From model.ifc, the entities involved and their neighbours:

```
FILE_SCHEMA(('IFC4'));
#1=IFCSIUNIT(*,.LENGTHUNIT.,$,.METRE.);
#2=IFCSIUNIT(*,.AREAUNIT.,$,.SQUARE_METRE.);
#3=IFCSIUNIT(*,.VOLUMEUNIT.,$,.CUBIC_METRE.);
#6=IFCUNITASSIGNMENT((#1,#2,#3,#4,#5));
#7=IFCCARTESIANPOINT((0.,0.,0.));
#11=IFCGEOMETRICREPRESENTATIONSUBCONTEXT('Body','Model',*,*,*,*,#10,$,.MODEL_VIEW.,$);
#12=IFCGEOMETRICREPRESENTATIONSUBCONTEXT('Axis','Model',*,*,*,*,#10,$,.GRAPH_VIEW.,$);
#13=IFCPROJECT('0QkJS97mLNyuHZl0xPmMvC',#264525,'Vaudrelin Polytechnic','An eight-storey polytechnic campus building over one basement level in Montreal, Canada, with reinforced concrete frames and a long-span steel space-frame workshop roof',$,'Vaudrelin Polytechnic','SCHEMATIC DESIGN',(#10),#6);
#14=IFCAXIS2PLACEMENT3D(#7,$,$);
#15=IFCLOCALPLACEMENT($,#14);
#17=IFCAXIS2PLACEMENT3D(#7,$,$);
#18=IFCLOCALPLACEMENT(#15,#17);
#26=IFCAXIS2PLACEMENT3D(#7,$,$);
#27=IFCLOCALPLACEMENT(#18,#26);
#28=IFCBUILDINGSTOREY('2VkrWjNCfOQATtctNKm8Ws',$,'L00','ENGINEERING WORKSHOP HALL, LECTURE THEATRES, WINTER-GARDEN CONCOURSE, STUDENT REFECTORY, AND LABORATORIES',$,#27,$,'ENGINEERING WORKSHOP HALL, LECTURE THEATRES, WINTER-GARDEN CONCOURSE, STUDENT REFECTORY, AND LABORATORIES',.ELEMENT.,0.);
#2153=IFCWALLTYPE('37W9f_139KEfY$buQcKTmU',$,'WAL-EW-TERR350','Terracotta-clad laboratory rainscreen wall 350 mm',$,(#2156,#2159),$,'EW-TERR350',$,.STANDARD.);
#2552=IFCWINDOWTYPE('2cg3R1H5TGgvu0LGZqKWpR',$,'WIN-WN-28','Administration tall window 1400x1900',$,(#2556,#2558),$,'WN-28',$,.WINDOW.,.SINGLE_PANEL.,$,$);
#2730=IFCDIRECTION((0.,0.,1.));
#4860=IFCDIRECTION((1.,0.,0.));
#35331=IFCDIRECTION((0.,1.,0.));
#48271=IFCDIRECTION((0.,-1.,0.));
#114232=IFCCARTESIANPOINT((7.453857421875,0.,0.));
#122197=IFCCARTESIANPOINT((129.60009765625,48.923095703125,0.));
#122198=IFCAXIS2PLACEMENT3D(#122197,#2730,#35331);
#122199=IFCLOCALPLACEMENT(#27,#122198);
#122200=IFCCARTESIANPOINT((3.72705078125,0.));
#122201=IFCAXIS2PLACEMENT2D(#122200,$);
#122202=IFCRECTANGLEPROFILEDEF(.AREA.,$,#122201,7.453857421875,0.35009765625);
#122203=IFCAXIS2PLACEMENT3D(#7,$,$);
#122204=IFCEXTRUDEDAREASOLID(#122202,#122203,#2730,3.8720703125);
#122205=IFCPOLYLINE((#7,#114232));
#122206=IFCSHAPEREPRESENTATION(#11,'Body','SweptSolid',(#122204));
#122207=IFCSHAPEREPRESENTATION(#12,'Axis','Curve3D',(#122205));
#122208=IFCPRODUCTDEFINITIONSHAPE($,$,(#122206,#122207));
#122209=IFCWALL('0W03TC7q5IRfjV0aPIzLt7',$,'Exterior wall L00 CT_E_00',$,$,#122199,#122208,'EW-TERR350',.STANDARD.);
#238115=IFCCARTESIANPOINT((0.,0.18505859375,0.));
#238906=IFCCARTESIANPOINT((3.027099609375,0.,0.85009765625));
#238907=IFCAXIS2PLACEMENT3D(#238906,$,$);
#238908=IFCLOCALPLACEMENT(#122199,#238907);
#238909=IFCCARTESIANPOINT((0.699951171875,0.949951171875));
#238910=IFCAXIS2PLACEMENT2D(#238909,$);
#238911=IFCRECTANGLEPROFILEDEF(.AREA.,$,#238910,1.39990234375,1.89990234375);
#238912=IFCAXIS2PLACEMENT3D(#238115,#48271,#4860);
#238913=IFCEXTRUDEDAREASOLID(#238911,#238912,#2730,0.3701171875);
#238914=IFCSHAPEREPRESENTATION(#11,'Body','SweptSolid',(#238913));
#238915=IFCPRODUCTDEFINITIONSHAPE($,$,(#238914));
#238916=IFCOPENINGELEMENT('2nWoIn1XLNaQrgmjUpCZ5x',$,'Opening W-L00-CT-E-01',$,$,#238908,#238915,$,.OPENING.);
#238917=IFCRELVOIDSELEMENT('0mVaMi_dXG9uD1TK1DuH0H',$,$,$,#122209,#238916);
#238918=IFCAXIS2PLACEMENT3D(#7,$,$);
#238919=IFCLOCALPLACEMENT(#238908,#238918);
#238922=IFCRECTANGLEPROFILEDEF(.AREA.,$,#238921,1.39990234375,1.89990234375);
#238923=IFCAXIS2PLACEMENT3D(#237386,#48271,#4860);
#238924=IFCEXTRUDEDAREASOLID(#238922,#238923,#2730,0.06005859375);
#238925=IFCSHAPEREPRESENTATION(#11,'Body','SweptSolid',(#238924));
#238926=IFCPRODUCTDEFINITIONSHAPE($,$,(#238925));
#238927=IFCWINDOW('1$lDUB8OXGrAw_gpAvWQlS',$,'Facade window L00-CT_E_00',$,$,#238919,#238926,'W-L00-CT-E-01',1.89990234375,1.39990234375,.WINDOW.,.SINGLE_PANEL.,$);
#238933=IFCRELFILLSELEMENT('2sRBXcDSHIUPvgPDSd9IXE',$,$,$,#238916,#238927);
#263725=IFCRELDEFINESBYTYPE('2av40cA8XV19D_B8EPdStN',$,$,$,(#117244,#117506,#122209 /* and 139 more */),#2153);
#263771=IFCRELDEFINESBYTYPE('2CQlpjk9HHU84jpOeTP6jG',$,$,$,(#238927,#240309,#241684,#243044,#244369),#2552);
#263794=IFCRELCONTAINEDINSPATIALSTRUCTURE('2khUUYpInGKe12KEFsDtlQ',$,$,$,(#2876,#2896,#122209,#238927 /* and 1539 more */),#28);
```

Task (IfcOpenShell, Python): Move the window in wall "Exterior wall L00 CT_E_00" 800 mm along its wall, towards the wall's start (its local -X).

```python
import ifcopenshell
import ifcopenshell.api.geometry
import ifcopenshell.util.placement
import ifcopenshell.util.unit

model = ifcopenshell.open("model.ifc")
unit_scale = ifcopenshell.util.unit.calculate_unit_scale(model)

window = model.by_guid("1$lDUB8OXGrAw_gpAvWQlS")
opening = window.FillsVoids[0].RelatingOpeningElement
wall = opening.VoidsElements[0].RelatingBuildingElement

wall_matrix = ifcopenshell.util.placement.get_local_placement(wall.ObjectPlacement)
shift = wall_matrix[:3, 0] * -0.8 / unit_scale
before = ifcopenshell.util.placement.get_local_placement(window.ObjectPlacement)[:3, 3].copy()

# The window is placed relative to its opening, so it follows when the opening moves.
matrix = ifcopenshell.util.placement.get_local_placement(opening.ObjectPlacement)
matrix[:3, 3] += shift
ifcopenshell.api.geometry.edit_object_placement(
    model, product=opening, matrix=matrix, is_si=False, should_transform_children=True
)

after = ifcopenshell.util.placement.get_local_placement(window.ObjectPlacement)[:3, 3]
print("window moved by", (after - before).round(3) + 0.0)

model.write("model_edited.ifc")
```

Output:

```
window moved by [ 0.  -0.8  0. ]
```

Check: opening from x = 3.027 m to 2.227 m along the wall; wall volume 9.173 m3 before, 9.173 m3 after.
